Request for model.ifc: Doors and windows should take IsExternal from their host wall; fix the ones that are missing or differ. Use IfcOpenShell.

First a look at what the model holds.

```python
import ifcopenshell
import ifcopenshell.util.element

model = ifcopenshell.open("model.ifc")
print(model.schema)
seen = {}
for e in model.by_type("IfcDoor") + model.by_type("IfcWindow"):
    if not e.FillsVoids:
        continue
    host = e.FillsVoids[0].RelatingOpeningElement.VoidsElements[0].RelatingBuildingElement
    own = ifcopenshell.util.element.get_pset(e, f"Pset_{e.is_a()[3:].removesuffix('StandardCase')}Common", "IsExternal")
    wall = ifcopenshell.util.element.get_pset(host, "Pset_WallCommon", "IsExternal")
    seen[e.is_a(), own, wall] = seen.get((e.is_a(), own, wall), 0) + 1
for (cls, own, wall), count in sorted(seen.items(), key=str):
    print(count, cls, "IsExternal:", own, "| host wall:", wall)
```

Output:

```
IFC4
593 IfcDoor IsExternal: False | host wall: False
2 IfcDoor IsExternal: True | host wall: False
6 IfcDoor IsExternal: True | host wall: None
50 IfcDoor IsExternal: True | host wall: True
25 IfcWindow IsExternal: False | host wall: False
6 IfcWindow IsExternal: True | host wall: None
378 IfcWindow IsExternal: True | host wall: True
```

```python
import ifcopenshell
import ifcopenshell.api.pset
import ifcopenshell.util.element

model = ifcopenshell.open("model.ifc")

count = 0
for ifc_class, pset_name in (("IfcDoor", "Pset_DoorCommon"), ("IfcWindow", "Pset_WindowCommon")):
    for e in model.by_type(ifc_class):
        if not e.FillsVoids:
            continue
        host = e.FillsVoids[0].RelatingOpeningElement.VoidsElements[0].RelatingBuildingElement
        external = ifcopenshell.util.element.get_pset(host, "Pset_WallCommon", "IsExternal")
        if external is None or ifcopenshell.util.element.get_pset(e, pset_name, "IsExternal") == external:
            continue
        pset = ifcopenshell.api.pset.add_pset(model, product=e, name=pset_name)
        ifcopenshell.api.pset.edit_pset(model, pset=pset, properties={"IsExternal": external})
        count += 1

print(count, "updated")

model.write("model_updated.ifc")
```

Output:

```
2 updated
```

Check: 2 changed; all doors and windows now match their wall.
